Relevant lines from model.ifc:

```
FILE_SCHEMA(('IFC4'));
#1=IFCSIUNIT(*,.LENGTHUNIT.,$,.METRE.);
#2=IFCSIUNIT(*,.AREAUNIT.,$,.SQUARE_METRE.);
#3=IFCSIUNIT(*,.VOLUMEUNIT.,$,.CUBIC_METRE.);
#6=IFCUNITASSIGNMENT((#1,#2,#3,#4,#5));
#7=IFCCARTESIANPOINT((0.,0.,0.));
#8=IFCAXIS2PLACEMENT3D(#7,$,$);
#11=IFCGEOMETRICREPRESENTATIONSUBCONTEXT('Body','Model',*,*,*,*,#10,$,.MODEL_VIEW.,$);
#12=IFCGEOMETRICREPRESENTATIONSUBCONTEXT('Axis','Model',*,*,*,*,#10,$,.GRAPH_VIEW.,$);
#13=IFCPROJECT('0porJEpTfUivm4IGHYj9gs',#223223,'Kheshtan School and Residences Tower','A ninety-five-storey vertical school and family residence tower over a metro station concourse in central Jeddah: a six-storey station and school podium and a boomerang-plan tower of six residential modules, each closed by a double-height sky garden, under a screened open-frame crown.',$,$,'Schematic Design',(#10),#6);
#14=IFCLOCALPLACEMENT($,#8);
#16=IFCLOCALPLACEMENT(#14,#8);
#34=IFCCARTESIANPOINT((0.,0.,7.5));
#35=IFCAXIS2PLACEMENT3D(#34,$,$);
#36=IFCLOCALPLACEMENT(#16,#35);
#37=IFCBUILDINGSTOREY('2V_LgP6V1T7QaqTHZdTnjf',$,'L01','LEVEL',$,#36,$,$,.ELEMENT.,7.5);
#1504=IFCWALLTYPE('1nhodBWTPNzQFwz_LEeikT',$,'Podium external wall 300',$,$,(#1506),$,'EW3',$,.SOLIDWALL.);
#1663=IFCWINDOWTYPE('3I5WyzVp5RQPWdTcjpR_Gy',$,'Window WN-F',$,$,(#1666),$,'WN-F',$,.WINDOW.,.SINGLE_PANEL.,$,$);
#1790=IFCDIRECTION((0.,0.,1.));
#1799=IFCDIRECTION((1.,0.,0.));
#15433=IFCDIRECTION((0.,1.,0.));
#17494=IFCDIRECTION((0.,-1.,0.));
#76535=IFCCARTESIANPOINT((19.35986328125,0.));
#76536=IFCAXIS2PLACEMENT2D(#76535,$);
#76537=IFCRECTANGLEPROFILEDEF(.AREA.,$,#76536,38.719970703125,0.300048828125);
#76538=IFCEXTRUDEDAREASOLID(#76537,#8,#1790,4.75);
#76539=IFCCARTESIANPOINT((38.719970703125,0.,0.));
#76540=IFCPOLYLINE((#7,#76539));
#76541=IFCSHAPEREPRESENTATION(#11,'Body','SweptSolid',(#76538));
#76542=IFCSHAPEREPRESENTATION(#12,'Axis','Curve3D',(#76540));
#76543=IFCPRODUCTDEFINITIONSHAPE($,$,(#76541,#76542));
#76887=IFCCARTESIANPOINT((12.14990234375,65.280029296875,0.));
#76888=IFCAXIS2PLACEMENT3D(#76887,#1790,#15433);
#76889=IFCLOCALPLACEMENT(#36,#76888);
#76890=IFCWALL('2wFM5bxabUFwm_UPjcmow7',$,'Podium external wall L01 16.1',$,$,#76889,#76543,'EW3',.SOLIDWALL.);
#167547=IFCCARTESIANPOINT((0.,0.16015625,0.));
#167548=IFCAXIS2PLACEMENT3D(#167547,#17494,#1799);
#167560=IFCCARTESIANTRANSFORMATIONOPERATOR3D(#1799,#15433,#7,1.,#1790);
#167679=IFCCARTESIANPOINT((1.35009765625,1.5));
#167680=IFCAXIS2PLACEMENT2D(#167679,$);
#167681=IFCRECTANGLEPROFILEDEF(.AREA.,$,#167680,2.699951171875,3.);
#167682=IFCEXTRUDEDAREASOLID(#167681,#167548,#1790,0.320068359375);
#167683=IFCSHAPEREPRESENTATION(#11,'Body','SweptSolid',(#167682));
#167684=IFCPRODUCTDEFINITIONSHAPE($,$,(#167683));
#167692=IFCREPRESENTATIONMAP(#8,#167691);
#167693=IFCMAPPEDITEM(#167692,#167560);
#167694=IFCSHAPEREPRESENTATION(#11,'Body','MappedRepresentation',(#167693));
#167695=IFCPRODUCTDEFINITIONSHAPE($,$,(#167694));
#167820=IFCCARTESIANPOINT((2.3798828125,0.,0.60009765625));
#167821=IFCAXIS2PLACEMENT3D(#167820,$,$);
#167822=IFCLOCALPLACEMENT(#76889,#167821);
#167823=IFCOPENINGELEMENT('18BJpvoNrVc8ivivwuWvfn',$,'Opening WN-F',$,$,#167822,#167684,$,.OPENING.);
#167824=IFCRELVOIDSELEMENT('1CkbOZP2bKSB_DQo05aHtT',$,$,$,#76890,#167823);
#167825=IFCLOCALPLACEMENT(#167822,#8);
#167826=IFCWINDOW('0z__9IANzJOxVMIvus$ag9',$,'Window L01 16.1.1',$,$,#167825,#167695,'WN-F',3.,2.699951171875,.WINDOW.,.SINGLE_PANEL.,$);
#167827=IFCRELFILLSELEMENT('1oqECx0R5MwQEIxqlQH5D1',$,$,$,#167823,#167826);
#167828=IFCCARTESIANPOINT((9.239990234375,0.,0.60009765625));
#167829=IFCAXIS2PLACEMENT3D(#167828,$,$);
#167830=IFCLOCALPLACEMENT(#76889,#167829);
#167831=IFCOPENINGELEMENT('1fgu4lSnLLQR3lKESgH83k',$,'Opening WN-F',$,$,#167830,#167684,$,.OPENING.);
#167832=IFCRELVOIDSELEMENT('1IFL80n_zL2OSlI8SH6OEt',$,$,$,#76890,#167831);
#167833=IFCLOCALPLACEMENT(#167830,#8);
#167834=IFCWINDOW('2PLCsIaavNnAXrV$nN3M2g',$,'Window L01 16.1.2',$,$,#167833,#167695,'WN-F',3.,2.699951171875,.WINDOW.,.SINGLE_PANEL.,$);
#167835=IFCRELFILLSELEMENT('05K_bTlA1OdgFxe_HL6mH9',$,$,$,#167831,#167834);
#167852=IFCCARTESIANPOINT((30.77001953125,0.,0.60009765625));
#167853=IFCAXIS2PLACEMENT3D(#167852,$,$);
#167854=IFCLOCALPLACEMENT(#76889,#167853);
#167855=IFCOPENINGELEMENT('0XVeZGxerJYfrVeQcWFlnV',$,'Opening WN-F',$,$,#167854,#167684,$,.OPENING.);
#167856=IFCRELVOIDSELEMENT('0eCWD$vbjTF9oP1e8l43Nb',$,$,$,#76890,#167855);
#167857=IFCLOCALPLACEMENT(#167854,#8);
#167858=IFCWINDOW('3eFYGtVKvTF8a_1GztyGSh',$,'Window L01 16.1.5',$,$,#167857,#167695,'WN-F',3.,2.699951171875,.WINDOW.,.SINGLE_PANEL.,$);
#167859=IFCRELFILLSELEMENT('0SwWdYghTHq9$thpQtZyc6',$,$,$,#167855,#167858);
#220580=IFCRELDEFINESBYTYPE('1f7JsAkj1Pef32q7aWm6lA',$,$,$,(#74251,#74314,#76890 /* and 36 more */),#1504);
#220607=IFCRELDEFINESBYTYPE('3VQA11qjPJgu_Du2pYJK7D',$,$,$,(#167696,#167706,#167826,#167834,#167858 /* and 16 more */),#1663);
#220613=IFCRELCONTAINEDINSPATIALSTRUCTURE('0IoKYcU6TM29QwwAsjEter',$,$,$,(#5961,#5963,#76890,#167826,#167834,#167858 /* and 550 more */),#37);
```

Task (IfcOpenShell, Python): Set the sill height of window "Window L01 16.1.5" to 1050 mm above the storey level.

```python
import numpy as np
import ifcopenshell
import ifcopenshell.api.geometry
import ifcopenshell.geom
import ifcopenshell.util.element
import ifcopenshell.util.placement
import ifcopenshell.util.shape
import ifcopenshell.util.unit

model = ifcopenshell.open("model.ifc")
unit_scale = ifcopenshell.util.unit.calculate_unit_scale(model)

window = model.by_guid("3eFYGtVKvTF8a_1GztyGSh")
opening = window.FillsVoids[0].RelatingOpeningElement
storey = ifcopenshell.util.element.get_container(window, ifc_class="IfcBuildingStorey")
level = ifcopenshell.util.placement.get_local_placement(storey.ObjectPlacement)[2, 3]

# The opening's origin need not be at the sill, so measure its lowest point.
shape = ifcopenshell.geom.create_shape(ifcopenshell.geom.settings(), opening)
bottom = ifcopenshell.util.shape.get_shape_bottom_elevation(shape, shape.geometry) / unit_scale
dz = level + 1.05 / unit_scale - bottom

shift = np.array([0.0, 0.0, dz])
# The window is placed relative to its opening, so it follows when the opening moves.
matrix = ifcopenshell.util.placement.get_local_placement(opening.ObjectPlacement)
matrix[:3, 3] += shift
ifcopenshell.api.geometry.edit_object_placement(
    model, product=opening, matrix=matrix, is_si=False, should_transform_children=True
)

print(f"moved by {dz * unit_scale:+.3f} m")

model.write("model_v2.ifc")
```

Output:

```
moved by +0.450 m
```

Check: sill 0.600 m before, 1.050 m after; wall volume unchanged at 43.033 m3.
